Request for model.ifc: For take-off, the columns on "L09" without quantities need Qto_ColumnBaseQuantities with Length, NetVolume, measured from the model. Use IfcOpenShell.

First a look at what the model holds.

```python
import ifcopenshell
import ifcopenshell.util.element
import ifcopenshell.util.unit

model = ifcopenshell.open("model.ifc")
print(model.schema)
for unit_type in ("LENGTHUNIT", "AREAUNIT", "VOLUMEUNIT"):
    print(unit_type, ifcopenshell.util.unit.calculate_unit_scale(model, unit_type))
storey = next(s for s in model.by_type("IfcBuildingStorey") if s.Name == "L09")
columns = [e for e in ifcopenshell.util.element.get_decomposition(storey) if e.is_a("IfcColumn")]
for e in sorted(columns, key=lambda e: e.id()):
    print(e.id(), e.is_a(), e.Name, list(ifcopenshell.util.element.get_psets(e, qtos_only=True)), sep=" | ")
```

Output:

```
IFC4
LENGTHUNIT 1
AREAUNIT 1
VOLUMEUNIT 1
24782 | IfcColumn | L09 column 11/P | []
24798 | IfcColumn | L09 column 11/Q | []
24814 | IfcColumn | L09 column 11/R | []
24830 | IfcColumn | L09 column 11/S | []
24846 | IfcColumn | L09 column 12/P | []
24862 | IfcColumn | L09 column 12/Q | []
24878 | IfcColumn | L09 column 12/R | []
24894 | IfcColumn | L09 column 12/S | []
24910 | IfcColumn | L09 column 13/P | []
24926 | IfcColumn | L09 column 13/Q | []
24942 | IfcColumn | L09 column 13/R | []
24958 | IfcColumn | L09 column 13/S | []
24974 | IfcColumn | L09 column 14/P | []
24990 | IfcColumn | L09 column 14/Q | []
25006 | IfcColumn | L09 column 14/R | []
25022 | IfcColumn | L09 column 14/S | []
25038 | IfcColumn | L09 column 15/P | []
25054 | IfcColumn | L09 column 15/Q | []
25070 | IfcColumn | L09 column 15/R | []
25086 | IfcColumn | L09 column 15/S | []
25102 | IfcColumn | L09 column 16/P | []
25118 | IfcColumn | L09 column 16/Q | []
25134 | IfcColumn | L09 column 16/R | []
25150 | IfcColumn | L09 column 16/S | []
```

```python
import ifcopenshell
import ifcopenshell.api.pset
import ifcopenshell.geom
import ifcopenshell.util.element
import ifcopenshell.util.shape
import ifcopenshell.util.unit

model = ifcopenshell.open("model.ifc")
unit_scale = ifcopenshell.util.unit.calculate_unit_scale(model)
volume_scale = ifcopenshell.util.unit.calculate_unit_scale(model, "VOLUMEUNIT")
settings = ifcopenshell.geom.settings()

storey = next(s for s in model.by_type("IfcBuildingStorey") if s.Name == "L09")
columns = [e for e in ifcopenshell.util.element.get_decomposition(storey) if e.is_a("IfcColumn")]

for e in sorted(columns, key=lambda e: e.id()):
    if ifcopenshell.util.element.get_psets(e, qtos_only=True, should_inherit=False):
        continue
    # Geometry comes back in metres, in the element's own axes.
    shape = ifcopenshell.geom.create_shape(settings, e)
    values = {
        "Length": ifcopenshell.util.shape.get_z(shape.geometry) / unit_scale,
        "NetVolume": ifcopenshell.util.shape.get_volume(shape.geometry) / volume_scale,
    }
    qto = ifcopenshell.api.pset.add_qto(model, product=e, name="Qto_ColumnBaseQuantities")
    ifcopenshell.api.pset.edit_qto(model, qto=qto, properties=values)
    print(e.id(), {k: round(v, 3) for k, v in values.items()})

model.write("model_v2.ifc")
```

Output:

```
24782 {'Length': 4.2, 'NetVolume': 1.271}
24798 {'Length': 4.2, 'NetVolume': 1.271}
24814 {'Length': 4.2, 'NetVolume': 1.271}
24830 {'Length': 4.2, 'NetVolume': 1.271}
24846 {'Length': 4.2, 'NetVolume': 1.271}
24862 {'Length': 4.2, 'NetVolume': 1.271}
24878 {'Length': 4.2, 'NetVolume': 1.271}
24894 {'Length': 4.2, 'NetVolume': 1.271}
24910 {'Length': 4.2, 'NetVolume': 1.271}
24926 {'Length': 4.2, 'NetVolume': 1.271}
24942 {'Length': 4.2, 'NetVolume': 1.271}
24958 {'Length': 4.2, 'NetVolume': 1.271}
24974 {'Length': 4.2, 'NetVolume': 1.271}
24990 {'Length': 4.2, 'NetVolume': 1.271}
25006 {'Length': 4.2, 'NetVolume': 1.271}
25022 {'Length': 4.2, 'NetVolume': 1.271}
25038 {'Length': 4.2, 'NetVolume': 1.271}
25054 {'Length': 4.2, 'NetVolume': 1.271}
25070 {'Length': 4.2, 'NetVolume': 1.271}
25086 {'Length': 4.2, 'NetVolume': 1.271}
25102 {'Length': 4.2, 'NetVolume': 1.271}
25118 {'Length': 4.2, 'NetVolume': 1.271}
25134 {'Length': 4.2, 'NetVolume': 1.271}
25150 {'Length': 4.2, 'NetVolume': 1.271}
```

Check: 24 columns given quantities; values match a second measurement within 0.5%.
